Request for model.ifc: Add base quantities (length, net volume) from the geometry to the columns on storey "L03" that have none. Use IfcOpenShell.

First a look at what the model holds.

```python
import ifcopenshell
import ifcopenshell.util.element
import ifcopenshell.util.unit

model = ifcopenshell.open("model.ifc")
print(model.schema)
for unit_type in ("LENGTHUNIT", "AREAUNIT", "VOLUMEUNIT"):
    print(unit_type, ifcopenshell.util.unit.calculate_unit_scale(model, unit_type))
storey = next(s for s in model.by_type("IfcBuildingStorey") if s.Name == "L03")
columns = [e for e in ifcopenshell.util.element.get_decomposition(storey) if e.is_a("IfcColumn")]
for e in sorted(columns, key=lambda e: e.id()):
    print(e.id(), e.is_a(), e.Name, list(ifcopenshell.util.element.get_psets(e, qtos_only=True)), sep=" | ")
```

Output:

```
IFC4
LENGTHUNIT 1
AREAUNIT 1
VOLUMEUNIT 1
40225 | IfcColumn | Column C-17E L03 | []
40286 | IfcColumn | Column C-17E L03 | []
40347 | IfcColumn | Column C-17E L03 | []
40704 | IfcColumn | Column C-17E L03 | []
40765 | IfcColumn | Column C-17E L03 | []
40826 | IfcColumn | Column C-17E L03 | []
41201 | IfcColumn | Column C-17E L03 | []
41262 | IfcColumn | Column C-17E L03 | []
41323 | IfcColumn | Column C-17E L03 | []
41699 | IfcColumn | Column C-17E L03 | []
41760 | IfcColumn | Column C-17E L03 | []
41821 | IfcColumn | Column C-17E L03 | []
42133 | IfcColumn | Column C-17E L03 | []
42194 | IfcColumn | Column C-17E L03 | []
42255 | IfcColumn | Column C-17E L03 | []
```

```python
import ifcopenshell
import ifcopenshell.api.pset
import ifcopenshell.geom
import ifcopenshell.util.element
import ifcopenshell.util.shape
import ifcopenshell.util.unit

model = ifcopenshell.open("model.ifc")
unit_scale = ifcopenshell.util.unit.calculate_unit_scale(model)
volume_scale = ifcopenshell.util.unit.calculate_unit_scale(model, "VOLUMEUNIT")
settings = ifcopenshell.geom.settings()

storey = next(s for s in model.by_type("IfcBuildingStorey") if s.Name == "L03")
columns = [e for e in ifcopenshell.util.element.get_decomposition(storey) if e.is_a("IfcColumn")]

for e in sorted(columns, key=lambda e: e.id()):
    if ifcopenshell.util.element.get_psets(e, qtos_only=True, should_inherit=False):
        continue
    # Geometry comes back in metres, in the element's own axes.
    shape = ifcopenshell.geom.create_shape(settings, e)
    values = {
        "Length": ifcopenshell.util.shape.get_z(shape.geometry) / unit_scale,
        "NetVolume": ifcopenshell.util.shape.get_volume(shape.geometry) / volume_scale,
    }
    qto = ifcopenshell.api.pset.add_qto(model, product=e, name="Qto_ColumnBaseQuantities")
    ifcopenshell.api.pset.edit_qto(model, qto=qto, properties=values)
    print(e.id(), {k: round(v, 3) for k, v in values.items()})

model.write("model_rev.ifc")
```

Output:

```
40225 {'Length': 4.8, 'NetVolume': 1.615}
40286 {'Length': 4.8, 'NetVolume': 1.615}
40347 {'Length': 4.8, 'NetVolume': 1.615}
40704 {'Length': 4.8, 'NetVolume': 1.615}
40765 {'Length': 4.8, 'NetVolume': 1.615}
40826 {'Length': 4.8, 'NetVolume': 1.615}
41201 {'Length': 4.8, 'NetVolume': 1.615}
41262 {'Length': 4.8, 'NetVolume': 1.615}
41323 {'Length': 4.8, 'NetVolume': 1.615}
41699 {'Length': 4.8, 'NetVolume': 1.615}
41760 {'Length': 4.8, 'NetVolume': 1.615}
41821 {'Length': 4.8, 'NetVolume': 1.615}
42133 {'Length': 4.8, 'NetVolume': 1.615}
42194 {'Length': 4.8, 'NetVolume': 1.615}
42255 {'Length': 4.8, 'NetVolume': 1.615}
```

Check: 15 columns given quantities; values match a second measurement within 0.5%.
